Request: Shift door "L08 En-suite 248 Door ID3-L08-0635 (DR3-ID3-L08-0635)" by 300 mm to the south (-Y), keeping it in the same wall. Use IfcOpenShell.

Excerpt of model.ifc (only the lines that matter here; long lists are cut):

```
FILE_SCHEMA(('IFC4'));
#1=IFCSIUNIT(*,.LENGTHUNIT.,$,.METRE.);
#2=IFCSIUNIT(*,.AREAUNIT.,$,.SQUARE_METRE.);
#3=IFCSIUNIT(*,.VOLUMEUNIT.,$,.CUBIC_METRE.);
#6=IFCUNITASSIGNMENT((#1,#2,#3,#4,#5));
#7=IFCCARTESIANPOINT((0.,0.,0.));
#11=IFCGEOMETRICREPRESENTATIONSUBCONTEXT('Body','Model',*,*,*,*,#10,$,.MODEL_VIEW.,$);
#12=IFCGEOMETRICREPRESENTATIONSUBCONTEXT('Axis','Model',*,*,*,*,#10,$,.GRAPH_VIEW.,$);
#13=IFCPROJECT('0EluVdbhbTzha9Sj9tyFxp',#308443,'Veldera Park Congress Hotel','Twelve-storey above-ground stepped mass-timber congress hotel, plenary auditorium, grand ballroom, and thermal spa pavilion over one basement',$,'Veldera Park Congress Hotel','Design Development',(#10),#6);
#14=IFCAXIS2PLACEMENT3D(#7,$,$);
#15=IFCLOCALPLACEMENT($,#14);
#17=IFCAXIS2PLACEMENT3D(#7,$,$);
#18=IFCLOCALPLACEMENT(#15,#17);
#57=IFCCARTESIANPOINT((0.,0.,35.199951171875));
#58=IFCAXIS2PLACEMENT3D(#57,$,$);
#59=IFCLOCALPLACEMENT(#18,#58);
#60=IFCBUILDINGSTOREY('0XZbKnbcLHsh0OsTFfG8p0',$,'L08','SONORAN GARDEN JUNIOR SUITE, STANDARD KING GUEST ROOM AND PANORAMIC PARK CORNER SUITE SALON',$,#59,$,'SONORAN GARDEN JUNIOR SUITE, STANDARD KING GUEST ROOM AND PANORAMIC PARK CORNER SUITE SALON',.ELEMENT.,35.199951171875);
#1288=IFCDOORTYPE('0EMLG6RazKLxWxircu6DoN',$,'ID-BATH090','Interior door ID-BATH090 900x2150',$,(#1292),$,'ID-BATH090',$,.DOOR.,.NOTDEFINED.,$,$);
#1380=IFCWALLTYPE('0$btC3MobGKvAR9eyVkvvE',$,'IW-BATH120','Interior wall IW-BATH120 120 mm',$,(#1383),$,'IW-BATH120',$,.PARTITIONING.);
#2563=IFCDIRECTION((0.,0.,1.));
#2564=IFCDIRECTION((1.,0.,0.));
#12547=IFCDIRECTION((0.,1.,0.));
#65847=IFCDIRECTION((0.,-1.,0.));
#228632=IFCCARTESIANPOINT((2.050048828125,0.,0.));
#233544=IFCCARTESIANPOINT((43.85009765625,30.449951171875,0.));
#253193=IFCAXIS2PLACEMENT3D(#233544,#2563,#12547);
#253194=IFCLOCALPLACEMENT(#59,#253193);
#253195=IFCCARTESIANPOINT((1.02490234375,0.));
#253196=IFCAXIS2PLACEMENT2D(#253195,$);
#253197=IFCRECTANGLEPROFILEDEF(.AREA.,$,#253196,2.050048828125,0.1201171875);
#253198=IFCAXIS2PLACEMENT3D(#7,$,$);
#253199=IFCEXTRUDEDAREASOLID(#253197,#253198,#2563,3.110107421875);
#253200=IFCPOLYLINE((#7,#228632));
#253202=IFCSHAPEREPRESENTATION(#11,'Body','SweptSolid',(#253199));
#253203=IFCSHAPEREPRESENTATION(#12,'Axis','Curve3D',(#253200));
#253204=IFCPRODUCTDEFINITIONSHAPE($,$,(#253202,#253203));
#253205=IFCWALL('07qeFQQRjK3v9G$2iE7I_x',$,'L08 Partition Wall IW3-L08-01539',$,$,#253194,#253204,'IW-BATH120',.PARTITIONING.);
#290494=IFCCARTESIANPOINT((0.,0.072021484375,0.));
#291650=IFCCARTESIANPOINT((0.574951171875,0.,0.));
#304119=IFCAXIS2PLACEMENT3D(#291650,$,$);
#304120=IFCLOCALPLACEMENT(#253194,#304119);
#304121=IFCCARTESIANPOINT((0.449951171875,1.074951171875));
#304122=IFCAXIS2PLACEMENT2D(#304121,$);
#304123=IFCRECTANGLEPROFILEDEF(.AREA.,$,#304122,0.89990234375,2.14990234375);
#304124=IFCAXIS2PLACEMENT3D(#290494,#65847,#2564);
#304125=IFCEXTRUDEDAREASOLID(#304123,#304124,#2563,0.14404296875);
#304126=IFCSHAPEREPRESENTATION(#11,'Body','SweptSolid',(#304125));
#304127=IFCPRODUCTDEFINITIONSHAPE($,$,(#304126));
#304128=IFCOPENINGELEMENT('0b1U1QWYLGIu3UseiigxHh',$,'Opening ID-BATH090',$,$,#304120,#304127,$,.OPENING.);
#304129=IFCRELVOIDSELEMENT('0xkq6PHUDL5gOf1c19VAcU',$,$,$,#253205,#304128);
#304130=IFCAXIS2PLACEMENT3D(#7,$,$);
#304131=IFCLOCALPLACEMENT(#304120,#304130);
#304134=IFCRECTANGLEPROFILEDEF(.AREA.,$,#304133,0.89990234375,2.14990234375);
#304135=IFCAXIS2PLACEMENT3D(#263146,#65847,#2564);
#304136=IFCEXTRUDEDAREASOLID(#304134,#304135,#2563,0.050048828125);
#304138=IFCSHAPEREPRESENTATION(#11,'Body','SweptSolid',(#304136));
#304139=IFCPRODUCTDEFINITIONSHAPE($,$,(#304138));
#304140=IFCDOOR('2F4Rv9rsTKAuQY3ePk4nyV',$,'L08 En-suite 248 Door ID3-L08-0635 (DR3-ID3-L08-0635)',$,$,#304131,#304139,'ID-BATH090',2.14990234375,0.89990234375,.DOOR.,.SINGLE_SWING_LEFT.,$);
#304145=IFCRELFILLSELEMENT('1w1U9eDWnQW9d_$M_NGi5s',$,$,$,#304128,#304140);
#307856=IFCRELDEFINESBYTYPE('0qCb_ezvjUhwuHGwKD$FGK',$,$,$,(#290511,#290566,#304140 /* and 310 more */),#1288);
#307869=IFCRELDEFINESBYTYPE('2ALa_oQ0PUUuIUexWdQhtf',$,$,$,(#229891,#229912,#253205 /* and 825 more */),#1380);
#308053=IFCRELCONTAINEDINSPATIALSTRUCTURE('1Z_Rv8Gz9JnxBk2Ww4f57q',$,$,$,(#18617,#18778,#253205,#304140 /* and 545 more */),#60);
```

```python
import ifcopenshell
import ifcopenshell.api.geometry
import ifcopenshell.util.placement

model = ifcopenshell.open("model.ifc")

door = model.by_guid("2F4Rv9rsTKAuQY3ePk4nyV")
opening = door.FillsVoids[0].RelatingOpeningElement
wall = opening.VoidsElements[0].RelatingBuildingElement

wall_matrix = ifcopenshell.util.placement.get_local_placement(wall.ObjectPlacement)
shift = wall_matrix[:3, 0] * -0.3
before = ifcopenshell.util.placement.get_local_placement(door.ObjectPlacement)[:3, 3].copy()

# The door is placed relative to its opening, so it follows when the opening moves.
matrix = ifcopenshell.util.placement.get_local_placement(opening.ObjectPlacement)
matrix[:3, 3] += shift
ifcopenshell.api.geometry.edit_object_placement(
    model, product=opening, matrix=matrix, is_si=False, should_transform_children=True
)

after = ifcopenshell.util.placement.get_local_placement(door.ObjectPlacement)[:3, 3]
print("door moved by", (after - before).round(3) + 0.0)

model.write("model_edited.ifc")
```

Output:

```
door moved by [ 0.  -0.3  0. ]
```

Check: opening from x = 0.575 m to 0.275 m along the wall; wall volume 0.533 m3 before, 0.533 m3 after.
